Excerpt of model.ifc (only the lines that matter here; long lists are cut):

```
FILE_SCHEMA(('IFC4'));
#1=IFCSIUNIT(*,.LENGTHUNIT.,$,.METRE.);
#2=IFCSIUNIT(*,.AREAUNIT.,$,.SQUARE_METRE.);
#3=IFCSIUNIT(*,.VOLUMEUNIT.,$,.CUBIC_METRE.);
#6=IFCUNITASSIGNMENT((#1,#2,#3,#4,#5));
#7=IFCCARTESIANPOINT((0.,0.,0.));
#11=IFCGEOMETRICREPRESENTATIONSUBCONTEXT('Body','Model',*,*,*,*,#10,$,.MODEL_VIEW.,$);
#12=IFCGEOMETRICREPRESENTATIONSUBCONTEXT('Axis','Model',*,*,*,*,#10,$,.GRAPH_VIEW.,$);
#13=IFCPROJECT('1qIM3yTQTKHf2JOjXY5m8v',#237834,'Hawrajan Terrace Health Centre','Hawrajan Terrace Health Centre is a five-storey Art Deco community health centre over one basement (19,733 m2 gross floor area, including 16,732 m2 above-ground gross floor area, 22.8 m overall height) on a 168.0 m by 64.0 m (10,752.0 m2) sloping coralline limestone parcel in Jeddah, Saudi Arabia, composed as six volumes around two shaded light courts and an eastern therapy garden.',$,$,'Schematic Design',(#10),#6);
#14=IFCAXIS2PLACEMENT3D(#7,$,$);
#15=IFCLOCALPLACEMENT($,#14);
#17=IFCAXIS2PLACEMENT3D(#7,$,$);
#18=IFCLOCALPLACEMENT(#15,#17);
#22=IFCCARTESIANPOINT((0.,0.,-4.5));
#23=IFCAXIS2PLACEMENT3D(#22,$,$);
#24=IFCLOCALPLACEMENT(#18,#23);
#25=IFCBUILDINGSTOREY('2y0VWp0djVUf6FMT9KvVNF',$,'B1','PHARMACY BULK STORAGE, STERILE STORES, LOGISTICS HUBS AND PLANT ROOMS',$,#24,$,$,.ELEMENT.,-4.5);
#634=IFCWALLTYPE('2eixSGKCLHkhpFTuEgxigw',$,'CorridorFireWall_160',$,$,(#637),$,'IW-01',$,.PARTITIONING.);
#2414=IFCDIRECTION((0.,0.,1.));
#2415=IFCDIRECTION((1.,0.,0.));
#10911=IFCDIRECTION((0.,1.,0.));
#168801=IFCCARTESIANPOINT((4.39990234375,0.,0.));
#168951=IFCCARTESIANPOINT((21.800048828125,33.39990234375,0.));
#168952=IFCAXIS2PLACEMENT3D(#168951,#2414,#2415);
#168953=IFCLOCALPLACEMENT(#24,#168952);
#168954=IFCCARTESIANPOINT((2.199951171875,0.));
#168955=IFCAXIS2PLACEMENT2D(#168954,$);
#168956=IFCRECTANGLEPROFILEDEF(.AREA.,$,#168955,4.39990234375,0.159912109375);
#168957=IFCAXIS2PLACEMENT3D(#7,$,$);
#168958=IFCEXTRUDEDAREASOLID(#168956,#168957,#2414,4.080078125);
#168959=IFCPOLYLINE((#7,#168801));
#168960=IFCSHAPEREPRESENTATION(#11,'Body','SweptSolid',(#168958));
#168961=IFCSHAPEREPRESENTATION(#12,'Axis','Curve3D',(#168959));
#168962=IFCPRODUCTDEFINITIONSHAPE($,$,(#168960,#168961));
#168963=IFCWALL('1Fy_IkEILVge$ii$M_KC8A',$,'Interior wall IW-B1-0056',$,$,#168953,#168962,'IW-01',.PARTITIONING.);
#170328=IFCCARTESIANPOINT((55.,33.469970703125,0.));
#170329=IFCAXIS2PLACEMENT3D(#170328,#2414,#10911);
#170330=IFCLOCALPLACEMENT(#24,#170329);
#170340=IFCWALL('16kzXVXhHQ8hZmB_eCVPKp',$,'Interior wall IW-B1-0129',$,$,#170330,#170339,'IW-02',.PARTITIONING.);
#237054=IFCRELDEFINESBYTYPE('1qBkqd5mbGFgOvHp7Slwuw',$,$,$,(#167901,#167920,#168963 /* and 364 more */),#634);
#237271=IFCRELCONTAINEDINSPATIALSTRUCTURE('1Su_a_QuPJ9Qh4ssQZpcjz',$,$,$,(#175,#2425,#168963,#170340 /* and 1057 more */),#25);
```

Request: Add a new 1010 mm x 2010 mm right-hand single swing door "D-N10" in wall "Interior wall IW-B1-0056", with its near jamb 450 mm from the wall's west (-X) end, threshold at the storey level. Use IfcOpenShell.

```python
import numpy as np
import ifcopenshell
import ifcopenshell.api.feature
import ifcopenshell.api.geometry
import ifcopenshell.api.root
import ifcopenshell.api.spatial
import ifcopenshell.geom
import ifcopenshell.util.element
import ifcopenshell.util.placement
import ifcopenshell.util.representation
import ifcopenshell.util.shape
import ifcopenshell.util.unit

model = ifcopenshell.open("model.ifc")
unit_scale = ifcopenshell.util.unit.calculate_unit_scale(model)
settings = ifcopenshell.geom.settings()


def volume(element):
    """Net volume in cubic metres, openings subtracted."""
    shape = ifcopenshell.geom.create_shape(settings, element)
    return ifcopenshell.util.shape.get_volume(shape.geometry)


wall = model.by_guid("1Fy_IkEILVge$ii$M_KC8A")
storey = ifcopenshell.util.element.get_container(wall, ifc_class="IfcBuildingStorey")
context = ifcopenshell.util.representation.get_context(model, "Model", "Body", "MODEL_VIEW")
before = volume(wall)

width, height, from_end, sill = 1.01, 2.01, 0.45, 0.0  # metres

# The wall runs along its own X axis, and the end named is its -X end.
wall_shape = ifcopenshell.geom.create_shape(settings, wall)
x, y, z = ifcopenshell.util.shape.get_vertices(wall_shape.geometry).T
start = x.min() + from_end
face, thickness = float(y.min()), float(y.max() - y.min())
wall_matrix = ifcopenshell.util.placement.get_local_placement(wall.ObjectPlacement)
level = ifcopenshell.util.placement.get_local_placement(storey.ObjectPlacement)[2, 3]


def in_wall(x, y):
    """Placement at x, y metres in the wall's axes, at sill height."""
    matrix = wall_matrix.copy()
    matrix[:, 3] = wall_matrix @ np.array([x / unit_scale, y / unit_scale, 0.0, 1.0])
    matrix[2, 3] = level + sill / unit_scale
    return matrix


# Opening: a box that overshoots both wall faces by 50 mm.
opening = ifcopenshell.api.root.create_entity(model, ifc_class="IfcOpeningElement", predefined_type="OPENING")
box = ifcopenshell.api.geometry.add_wall_representation(
    model, context=context, length=width, height=height, thickness=thickness + 0.1
)
ifcopenshell.api.geometry.assign_representation(model, product=opening, representation=box)
ifcopenshell.api.geometry.edit_object_placement(model, product=opening, matrix=in_wall(start, face - 0.05), is_si=False)
ifcopenshell.api.feature.add_feature(model, feature=opening, element=wall)

door = ifcopenshell.api.root.create_entity(model, ifc_class="IfcDoor", name="D-N10", predefined_type="DOOR")
door.OverallWidth, door.OverallHeight = width / unit_scale, height / unit_scale
door.OperationType = "SINGLE_SWING_RIGHT"
body = ifcopenshell.api.geometry.add_door_representation(
    model,
    context=context,
    overall_width=door.OverallWidth,
    overall_height=door.OverallHeight,
    operation_type="SINGLE_SWING_RIGHT",
    lining_properties={"LiningDepth": thickness / unit_scale, "ThresholdDepth": thickness / unit_scale},
)
ifcopenshell.api.geometry.assign_representation(model, product=door, representation=body)
ifcopenshell.api.spatial.assign_container(model, products=[door], relating_structure=storey)
ifcopenshell.api.feature.add_filling(model, opening=opening, element=door)

# The lining spans the wall, so the door starts at the wall face.
ifcopenshell.api.geometry.edit_object_placement(model, product=door, matrix=in_wall(start, face), is_si=False)

after = volume(wall)

print(f"wall volume {before:.3f} -> {after:.3f} m3")

model.write("model_edited.ifc")
```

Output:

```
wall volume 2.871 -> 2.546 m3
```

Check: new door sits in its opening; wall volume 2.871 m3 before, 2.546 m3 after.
